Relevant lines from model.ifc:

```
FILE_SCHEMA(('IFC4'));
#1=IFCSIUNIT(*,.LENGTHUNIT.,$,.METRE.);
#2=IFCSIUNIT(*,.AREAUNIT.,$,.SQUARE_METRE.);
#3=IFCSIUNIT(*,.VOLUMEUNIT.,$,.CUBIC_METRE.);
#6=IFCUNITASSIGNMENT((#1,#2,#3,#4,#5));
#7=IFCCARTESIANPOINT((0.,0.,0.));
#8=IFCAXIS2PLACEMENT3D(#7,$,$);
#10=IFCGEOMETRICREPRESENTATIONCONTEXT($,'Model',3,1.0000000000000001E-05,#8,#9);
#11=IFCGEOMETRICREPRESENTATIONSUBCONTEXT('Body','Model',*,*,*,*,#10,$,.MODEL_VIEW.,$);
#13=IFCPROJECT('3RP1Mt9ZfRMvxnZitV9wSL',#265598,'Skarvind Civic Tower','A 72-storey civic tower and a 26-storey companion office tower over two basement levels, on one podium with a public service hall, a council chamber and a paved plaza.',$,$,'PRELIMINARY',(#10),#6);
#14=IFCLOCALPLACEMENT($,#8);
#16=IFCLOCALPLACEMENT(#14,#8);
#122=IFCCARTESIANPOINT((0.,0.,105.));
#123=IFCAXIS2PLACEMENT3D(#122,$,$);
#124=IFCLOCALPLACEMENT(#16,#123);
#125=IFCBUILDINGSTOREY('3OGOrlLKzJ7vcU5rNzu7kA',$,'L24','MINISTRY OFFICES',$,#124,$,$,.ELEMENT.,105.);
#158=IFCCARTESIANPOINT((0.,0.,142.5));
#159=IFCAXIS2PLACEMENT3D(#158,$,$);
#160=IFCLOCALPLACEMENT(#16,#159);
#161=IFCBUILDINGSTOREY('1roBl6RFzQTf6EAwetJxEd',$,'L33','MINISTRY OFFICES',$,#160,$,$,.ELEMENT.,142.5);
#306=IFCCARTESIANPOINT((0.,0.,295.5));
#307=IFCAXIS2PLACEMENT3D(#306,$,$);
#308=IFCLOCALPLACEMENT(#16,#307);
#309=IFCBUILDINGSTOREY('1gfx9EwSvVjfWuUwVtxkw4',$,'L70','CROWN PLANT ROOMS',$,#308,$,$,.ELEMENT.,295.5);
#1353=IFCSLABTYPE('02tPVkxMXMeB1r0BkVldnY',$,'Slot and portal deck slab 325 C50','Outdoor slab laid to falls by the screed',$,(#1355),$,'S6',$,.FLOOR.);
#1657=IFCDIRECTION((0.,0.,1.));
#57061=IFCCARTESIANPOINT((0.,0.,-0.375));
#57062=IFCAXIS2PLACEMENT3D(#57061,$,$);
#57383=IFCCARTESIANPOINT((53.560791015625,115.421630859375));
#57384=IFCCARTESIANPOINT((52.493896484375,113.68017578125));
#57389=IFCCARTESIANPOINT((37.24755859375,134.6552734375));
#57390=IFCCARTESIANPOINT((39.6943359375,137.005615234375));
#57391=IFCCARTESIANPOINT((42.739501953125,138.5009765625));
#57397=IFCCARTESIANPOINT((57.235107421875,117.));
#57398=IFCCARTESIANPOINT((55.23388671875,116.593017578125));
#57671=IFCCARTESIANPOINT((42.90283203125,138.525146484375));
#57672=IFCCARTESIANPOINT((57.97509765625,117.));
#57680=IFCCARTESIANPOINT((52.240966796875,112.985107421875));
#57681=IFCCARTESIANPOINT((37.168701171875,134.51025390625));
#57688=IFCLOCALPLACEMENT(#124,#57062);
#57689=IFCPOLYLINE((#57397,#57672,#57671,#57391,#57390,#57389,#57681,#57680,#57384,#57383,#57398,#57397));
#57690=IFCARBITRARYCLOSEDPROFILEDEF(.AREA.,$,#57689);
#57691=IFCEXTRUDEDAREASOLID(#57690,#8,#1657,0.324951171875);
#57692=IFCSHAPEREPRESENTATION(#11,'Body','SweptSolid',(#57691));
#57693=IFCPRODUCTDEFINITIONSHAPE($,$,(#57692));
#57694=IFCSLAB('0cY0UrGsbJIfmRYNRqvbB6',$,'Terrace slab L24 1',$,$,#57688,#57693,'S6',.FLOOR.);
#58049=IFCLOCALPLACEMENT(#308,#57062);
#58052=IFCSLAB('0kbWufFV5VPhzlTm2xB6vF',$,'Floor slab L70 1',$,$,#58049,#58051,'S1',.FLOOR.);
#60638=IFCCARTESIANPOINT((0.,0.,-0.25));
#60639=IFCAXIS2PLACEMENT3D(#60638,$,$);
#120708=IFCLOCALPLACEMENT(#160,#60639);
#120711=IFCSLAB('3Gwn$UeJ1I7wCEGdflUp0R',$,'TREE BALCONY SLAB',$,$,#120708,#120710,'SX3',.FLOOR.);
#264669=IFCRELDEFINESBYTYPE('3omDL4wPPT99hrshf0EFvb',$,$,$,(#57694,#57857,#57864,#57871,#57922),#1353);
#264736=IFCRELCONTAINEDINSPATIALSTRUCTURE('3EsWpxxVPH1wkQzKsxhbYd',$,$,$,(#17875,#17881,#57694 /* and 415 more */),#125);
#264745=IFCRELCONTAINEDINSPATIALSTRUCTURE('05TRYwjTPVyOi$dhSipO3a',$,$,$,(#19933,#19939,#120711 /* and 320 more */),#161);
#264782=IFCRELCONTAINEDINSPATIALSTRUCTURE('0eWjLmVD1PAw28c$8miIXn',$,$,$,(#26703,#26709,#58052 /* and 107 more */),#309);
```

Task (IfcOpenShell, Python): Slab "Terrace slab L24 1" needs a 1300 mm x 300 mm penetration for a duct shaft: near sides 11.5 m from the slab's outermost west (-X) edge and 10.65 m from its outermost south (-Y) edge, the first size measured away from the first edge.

```python
import numpy as np
import ifcopenshell
import ifcopenshell.api.feature
import ifcopenshell.api.geometry
import ifcopenshell.api.root
import ifcopenshell.geom
import ifcopenshell.util.placement
import ifcopenshell.util.representation
import ifcopenshell.util.shape
import ifcopenshell.util.unit

model = ifcopenshell.open("model.ifc")
unit_scale = ifcopenshell.util.unit.calculate_unit_scale(model)
settings = ifcopenshell.geom.settings()


def volume(element):
    """Net volume in cubic metres, openings subtracted."""
    shape = ifcopenshell.geom.create_shape(settings, element)
    return ifcopenshell.util.shape.get_volume(shape.geometry)


slab = model.by_guid("0cY0UrGsbJIfmRYNRqvbB6")
before = volume(slab)

# Extent in the slab's own axes, in metres. The edges named are its -X and -Y sides.
slab_shape = ifcopenshell.geom.create_shape(settings, slab)
vertices = ifcopenshell.util.shape.get_vertices(slab_shape.geometry)
x_min, y_min, bottom = vertices.min(axis=0)
top = vertices[:, 2].max()

opening = ifcopenshell.api.root.create_entity(model, ifc_class="IfcOpeningElement", name="Duct shaft opening", predefined_type="OPENING")
context = ifcopenshell.util.representation.get_context(model, "Model", "Body", "MODEL_VIEW")
width, depth = 1.3, 0.3
outline = [(0.0, 0.0), (width, 0.0), (width, depth), (0.0, depth), (0.0, 0.0)]
# Overshoot both faces by 50 mm so the cut is clean.
shape = ifcopenshell.api.geometry.add_slab_representation(
    model, context=context, depth=top - bottom + 0.1, polyline=outline
)
ifcopenshell.api.geometry.assign_representation(model, product=opening, representation=shape)

matrix = ifcopenshell.util.placement.get_local_placement(slab.ObjectPlacement)
matrix[:, 3] = matrix @ np.append(np.array([x_min + 11.5, y_min + 10.65, bottom - 0.05]) / unit_scale, 1.0)
ifcopenshell.api.geometry.edit_object_placement(model, product=opening, matrix=matrix, is_si=False)
ifcopenshell.api.feature.add_feature(model, feature=opening, element=slab)

after = volume(slab)

print(f"slab volume {before:.3f} -> {after:.3f} m3")

model.write("model_updated.ifc")
```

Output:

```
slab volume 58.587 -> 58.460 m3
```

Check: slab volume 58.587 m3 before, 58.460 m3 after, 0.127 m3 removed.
